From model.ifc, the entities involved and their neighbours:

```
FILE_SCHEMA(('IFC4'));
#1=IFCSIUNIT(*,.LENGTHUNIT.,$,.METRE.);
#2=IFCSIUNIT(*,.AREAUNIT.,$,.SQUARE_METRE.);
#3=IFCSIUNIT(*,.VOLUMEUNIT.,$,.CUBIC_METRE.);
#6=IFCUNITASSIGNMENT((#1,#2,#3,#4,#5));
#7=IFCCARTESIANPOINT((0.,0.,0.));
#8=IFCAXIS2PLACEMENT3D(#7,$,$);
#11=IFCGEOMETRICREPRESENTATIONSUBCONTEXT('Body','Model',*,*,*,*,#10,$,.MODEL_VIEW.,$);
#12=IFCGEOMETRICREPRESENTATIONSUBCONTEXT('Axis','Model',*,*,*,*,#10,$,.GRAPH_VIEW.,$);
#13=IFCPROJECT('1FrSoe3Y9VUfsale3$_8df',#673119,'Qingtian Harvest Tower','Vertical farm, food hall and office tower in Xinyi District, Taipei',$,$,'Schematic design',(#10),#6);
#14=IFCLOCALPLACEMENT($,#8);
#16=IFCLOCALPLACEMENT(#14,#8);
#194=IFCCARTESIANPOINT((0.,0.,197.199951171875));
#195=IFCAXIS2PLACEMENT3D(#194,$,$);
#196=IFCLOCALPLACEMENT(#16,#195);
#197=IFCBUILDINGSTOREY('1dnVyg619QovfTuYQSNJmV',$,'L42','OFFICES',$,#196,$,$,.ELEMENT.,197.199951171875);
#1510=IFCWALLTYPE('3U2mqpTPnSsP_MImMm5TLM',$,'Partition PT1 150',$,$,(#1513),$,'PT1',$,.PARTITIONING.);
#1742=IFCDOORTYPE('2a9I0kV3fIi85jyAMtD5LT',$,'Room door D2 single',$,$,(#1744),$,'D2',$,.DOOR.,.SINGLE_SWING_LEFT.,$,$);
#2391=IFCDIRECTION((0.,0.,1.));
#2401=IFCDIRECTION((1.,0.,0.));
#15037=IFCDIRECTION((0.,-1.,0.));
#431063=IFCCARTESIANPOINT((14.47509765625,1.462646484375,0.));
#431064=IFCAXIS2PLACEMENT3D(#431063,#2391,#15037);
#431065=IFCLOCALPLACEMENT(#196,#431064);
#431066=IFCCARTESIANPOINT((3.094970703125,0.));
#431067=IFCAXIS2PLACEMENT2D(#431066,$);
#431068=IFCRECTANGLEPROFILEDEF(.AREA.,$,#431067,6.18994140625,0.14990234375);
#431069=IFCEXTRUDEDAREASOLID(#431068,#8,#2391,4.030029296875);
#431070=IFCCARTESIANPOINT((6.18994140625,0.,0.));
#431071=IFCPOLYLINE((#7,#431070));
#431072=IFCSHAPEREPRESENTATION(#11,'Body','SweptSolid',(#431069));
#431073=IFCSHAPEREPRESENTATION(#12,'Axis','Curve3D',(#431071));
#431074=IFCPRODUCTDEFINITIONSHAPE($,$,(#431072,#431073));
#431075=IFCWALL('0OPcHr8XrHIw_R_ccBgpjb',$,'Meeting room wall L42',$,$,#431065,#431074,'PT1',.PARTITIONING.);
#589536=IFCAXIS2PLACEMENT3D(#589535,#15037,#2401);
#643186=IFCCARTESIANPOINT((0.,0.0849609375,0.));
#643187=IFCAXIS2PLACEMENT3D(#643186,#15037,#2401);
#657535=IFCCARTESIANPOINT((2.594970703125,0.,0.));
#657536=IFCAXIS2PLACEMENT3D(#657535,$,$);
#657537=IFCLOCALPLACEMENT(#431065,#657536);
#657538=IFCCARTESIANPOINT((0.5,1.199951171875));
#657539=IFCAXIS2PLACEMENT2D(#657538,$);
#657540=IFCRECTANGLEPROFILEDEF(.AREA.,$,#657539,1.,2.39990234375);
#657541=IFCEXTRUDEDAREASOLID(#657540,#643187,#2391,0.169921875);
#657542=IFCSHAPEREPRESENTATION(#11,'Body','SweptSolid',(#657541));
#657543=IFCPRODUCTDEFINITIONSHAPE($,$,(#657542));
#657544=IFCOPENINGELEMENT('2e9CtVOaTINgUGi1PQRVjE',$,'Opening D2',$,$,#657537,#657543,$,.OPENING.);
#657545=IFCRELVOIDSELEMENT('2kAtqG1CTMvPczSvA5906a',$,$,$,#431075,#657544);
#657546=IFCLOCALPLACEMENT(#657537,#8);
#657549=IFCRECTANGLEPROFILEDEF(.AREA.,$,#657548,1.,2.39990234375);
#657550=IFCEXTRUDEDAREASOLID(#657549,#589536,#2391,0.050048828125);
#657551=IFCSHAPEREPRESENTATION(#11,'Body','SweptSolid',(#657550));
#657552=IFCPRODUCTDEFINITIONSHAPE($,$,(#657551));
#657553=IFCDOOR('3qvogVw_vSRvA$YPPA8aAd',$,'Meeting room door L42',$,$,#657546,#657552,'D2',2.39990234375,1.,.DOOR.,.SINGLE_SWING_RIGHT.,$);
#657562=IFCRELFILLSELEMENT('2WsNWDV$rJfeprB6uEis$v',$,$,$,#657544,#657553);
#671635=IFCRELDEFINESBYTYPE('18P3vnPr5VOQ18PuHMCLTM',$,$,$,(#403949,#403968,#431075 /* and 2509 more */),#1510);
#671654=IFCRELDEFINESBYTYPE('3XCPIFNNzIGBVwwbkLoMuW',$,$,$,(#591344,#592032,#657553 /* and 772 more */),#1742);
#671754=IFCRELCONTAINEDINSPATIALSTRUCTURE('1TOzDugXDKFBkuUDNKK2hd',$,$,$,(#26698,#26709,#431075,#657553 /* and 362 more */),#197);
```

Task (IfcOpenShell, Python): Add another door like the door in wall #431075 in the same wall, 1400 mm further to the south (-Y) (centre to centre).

```python
import ifcopenshell
import ifcopenshell.api.feature
import ifcopenshell.api.geometry
import ifcopenshell.api.root
import ifcopenshell.geom
import ifcopenshell.util.element
import ifcopenshell.util.placement
import ifcopenshell.util.shape
import ifcopenshell.util.unit

model = ifcopenshell.open("model.ifc")
unit_scale = ifcopenshell.util.unit.calculate_unit_scale(model)
settings = ifcopenshell.geom.settings()


def volume(element):
    """Net volume in cubic metres, openings subtracted."""
    shape = ifcopenshell.geom.create_shape(settings, element)
    return ifcopenshell.util.shape.get_volume(shape.geometry)


door = model.by_guid("3qvogVw_vSRvA$YPPA8aAd")
opening = door.FillsVoids[0].RelatingOpeningElement
wall = opening.VoidsElements[0].RelatingBuildingElement
before = volume(wall)
shift = ifcopenshell.util.placement.get_local_placement(wall.ObjectPlacement)[:3, 0] * 1.4 / unit_scale

# copy_class copies the void relationship, type, container and properties, but no geometry.
new_opening = ifcopenshell.api.root.copy_class(model, product=opening)
new_opening.Representation = ifcopenshell.util.element.copy_deep(
    model, opening.Representation, exclude=["IfcGeometricRepresentationContext", "IfcRepresentationMap"]
)
new_door = ifcopenshell.api.root.copy_class(model, product=door)
new_door.Representation = ifcopenshell.util.element.copy_deep(
    model, door.Representation, exclude=["IfcGeometricRepresentationContext", "IfcRepresentationMap"]
)
new_door.Tag = None
ifcopenshell.api.feature.add_filling(model, opening=new_opening, element=new_door)

for old, new in ((opening, new_opening), (door, new_door)):
    matrix = ifcopenshell.util.placement.get_local_placement(old.ObjectPlacement)
    matrix[:3, 3] += shift
    ifcopenshell.api.geometry.edit_object_placement(model, product=new, matrix=matrix, is_si=False)

after = volume(wall)

print(f"wall volume {before:.3f} -> {after:.3f} m3")

model.write("model_v2.ifc")
```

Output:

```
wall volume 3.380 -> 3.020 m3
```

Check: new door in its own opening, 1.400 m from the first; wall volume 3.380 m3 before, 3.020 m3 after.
